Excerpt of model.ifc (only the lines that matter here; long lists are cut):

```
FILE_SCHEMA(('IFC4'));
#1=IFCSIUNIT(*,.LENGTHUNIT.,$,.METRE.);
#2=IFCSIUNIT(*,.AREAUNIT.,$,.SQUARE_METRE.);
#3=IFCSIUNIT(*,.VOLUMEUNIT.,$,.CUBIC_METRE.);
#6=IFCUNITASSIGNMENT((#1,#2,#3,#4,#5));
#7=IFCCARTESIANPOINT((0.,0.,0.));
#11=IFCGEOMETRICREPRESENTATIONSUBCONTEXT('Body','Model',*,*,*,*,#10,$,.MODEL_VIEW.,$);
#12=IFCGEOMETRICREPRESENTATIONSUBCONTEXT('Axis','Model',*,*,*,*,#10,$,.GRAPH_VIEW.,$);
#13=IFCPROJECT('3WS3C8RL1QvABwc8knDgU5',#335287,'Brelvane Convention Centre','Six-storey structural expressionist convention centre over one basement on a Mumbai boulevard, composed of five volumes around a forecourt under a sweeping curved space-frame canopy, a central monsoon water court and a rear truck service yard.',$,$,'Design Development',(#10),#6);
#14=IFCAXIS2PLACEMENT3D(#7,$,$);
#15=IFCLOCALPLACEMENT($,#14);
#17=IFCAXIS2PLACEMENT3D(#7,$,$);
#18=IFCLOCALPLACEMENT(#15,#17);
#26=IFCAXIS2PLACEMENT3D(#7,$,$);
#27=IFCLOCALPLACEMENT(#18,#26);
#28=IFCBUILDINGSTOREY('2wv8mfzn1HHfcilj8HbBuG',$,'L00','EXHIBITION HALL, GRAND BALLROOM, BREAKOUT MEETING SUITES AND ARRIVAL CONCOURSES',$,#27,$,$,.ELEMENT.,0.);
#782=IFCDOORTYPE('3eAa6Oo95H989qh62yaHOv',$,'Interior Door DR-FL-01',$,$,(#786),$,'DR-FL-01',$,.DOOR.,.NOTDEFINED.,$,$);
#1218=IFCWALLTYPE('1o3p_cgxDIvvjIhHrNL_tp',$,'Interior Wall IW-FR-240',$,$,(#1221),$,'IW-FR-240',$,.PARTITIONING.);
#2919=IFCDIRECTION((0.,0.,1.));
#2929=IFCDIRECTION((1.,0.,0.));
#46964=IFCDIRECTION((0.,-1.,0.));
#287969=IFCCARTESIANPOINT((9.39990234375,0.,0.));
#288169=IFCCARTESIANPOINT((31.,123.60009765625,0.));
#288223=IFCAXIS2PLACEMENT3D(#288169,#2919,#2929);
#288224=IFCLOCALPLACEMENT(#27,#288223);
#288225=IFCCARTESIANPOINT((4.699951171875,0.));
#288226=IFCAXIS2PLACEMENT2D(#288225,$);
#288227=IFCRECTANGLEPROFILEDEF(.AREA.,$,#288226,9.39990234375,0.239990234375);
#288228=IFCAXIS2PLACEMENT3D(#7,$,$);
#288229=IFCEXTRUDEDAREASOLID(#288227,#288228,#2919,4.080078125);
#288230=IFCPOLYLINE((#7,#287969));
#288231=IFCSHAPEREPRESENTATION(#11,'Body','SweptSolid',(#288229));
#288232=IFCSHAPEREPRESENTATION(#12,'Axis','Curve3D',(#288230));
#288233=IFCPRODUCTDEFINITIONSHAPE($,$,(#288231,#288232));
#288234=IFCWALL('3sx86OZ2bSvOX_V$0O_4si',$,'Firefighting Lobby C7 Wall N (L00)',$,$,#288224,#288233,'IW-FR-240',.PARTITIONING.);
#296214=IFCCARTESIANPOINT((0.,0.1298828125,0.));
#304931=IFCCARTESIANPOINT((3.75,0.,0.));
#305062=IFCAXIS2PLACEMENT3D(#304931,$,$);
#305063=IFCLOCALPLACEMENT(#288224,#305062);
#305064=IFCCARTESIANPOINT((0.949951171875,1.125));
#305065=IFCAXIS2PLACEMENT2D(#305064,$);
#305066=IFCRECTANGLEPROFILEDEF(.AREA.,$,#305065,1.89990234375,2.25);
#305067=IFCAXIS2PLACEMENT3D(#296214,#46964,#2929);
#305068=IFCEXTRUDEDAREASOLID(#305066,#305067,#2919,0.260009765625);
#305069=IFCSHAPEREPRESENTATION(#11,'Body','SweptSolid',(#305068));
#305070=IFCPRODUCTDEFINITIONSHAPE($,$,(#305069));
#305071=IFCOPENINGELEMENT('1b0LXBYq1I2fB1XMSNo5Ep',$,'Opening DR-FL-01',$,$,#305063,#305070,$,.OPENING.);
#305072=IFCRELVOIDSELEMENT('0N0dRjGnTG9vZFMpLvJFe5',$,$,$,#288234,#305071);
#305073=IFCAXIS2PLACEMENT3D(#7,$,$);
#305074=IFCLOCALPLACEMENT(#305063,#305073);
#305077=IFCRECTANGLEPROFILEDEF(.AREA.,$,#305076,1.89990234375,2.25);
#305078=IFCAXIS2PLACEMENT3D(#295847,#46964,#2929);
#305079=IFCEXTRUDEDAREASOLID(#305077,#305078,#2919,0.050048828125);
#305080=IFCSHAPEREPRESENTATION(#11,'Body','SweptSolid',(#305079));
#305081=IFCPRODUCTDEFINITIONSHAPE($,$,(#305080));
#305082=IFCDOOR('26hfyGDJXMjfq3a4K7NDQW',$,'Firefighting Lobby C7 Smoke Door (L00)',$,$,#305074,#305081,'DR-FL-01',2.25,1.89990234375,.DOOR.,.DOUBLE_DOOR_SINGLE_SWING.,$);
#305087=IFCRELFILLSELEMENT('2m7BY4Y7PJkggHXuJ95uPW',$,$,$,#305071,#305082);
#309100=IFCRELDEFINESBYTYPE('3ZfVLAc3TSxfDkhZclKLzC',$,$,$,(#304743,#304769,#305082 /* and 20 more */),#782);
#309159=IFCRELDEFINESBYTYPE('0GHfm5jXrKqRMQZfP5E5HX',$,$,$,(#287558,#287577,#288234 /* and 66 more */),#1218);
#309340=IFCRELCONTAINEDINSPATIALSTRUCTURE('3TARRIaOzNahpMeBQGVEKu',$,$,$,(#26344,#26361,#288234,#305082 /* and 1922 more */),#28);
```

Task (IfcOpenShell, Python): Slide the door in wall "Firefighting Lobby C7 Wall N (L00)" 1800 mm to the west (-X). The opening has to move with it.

```python
import ifcopenshell
import ifcopenshell.api.geometry
import ifcopenshell.util.placement

model = ifcopenshell.open("model.ifc")

door = model.by_id(305082)
opening = door.FillsVoids[0].RelatingOpeningElement
wall = opening.VoidsElements[0].RelatingBuildingElement

wall_matrix = ifcopenshell.util.placement.get_local_placement(wall.ObjectPlacement)
shift = wall_matrix[:3, 0] * -1.8
before = ifcopenshell.util.placement.get_local_placement(door.ObjectPlacement)[:3, 3].copy()

# The door is placed relative to its opening, so it follows when the opening moves.
matrix = ifcopenshell.util.placement.get_local_placement(opening.ObjectPlacement)
matrix[:3, 3] += shift
ifcopenshell.api.geometry.edit_object_placement(
    model, product=opening, matrix=matrix, is_si=False, should_transform_children=True
)

after = ifcopenshell.util.placement.get_local_placement(door.ObjectPlacement)[:3, 3]
print("door moved by", (after - before).round(3) + 0.0)

model.write("model_rev.ifc")
```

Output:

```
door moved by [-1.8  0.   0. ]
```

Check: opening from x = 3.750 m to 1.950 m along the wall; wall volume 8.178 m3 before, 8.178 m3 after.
